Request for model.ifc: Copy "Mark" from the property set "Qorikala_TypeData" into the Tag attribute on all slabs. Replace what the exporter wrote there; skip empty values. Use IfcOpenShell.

First a look at what the model holds.

```python
import ifcopenshell
import ifcopenshell.util.element

model = ifcopenshell.open("model.ifc")
print(model.schema)
slabs = model.by_type("IfcSlab")
print(len(slabs), "slabs")
for e in slabs[:8]:
    source = ifcopenshell.util.element.get_pset(e, "Qorikala_TypeData", "Mark")
    target = e.Tag
    print(e.id(), repr(source), repr(target), sep=" | ")
```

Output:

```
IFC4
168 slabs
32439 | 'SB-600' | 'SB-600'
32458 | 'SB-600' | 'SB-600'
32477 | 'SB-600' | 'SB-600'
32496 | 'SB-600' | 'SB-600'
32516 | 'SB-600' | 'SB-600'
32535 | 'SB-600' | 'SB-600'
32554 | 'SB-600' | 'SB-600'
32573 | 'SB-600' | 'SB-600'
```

```python
import ifcopenshell
import ifcopenshell.util.element

model = ifcopenshell.open("model.ifc")

count = 0
for e in model.by_type("IfcSlab"):
    value = ifcopenshell.util.element.get_pset(e, "Qorikala_TypeData", "Mark")
    current = e.Tag
    if not value or not value.strip() or current == value:
        continue
    e.Tag = value
    count += 1

print(count, "slabs updated")

model.write("model_rev.ifc")
```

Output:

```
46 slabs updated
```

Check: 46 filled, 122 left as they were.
